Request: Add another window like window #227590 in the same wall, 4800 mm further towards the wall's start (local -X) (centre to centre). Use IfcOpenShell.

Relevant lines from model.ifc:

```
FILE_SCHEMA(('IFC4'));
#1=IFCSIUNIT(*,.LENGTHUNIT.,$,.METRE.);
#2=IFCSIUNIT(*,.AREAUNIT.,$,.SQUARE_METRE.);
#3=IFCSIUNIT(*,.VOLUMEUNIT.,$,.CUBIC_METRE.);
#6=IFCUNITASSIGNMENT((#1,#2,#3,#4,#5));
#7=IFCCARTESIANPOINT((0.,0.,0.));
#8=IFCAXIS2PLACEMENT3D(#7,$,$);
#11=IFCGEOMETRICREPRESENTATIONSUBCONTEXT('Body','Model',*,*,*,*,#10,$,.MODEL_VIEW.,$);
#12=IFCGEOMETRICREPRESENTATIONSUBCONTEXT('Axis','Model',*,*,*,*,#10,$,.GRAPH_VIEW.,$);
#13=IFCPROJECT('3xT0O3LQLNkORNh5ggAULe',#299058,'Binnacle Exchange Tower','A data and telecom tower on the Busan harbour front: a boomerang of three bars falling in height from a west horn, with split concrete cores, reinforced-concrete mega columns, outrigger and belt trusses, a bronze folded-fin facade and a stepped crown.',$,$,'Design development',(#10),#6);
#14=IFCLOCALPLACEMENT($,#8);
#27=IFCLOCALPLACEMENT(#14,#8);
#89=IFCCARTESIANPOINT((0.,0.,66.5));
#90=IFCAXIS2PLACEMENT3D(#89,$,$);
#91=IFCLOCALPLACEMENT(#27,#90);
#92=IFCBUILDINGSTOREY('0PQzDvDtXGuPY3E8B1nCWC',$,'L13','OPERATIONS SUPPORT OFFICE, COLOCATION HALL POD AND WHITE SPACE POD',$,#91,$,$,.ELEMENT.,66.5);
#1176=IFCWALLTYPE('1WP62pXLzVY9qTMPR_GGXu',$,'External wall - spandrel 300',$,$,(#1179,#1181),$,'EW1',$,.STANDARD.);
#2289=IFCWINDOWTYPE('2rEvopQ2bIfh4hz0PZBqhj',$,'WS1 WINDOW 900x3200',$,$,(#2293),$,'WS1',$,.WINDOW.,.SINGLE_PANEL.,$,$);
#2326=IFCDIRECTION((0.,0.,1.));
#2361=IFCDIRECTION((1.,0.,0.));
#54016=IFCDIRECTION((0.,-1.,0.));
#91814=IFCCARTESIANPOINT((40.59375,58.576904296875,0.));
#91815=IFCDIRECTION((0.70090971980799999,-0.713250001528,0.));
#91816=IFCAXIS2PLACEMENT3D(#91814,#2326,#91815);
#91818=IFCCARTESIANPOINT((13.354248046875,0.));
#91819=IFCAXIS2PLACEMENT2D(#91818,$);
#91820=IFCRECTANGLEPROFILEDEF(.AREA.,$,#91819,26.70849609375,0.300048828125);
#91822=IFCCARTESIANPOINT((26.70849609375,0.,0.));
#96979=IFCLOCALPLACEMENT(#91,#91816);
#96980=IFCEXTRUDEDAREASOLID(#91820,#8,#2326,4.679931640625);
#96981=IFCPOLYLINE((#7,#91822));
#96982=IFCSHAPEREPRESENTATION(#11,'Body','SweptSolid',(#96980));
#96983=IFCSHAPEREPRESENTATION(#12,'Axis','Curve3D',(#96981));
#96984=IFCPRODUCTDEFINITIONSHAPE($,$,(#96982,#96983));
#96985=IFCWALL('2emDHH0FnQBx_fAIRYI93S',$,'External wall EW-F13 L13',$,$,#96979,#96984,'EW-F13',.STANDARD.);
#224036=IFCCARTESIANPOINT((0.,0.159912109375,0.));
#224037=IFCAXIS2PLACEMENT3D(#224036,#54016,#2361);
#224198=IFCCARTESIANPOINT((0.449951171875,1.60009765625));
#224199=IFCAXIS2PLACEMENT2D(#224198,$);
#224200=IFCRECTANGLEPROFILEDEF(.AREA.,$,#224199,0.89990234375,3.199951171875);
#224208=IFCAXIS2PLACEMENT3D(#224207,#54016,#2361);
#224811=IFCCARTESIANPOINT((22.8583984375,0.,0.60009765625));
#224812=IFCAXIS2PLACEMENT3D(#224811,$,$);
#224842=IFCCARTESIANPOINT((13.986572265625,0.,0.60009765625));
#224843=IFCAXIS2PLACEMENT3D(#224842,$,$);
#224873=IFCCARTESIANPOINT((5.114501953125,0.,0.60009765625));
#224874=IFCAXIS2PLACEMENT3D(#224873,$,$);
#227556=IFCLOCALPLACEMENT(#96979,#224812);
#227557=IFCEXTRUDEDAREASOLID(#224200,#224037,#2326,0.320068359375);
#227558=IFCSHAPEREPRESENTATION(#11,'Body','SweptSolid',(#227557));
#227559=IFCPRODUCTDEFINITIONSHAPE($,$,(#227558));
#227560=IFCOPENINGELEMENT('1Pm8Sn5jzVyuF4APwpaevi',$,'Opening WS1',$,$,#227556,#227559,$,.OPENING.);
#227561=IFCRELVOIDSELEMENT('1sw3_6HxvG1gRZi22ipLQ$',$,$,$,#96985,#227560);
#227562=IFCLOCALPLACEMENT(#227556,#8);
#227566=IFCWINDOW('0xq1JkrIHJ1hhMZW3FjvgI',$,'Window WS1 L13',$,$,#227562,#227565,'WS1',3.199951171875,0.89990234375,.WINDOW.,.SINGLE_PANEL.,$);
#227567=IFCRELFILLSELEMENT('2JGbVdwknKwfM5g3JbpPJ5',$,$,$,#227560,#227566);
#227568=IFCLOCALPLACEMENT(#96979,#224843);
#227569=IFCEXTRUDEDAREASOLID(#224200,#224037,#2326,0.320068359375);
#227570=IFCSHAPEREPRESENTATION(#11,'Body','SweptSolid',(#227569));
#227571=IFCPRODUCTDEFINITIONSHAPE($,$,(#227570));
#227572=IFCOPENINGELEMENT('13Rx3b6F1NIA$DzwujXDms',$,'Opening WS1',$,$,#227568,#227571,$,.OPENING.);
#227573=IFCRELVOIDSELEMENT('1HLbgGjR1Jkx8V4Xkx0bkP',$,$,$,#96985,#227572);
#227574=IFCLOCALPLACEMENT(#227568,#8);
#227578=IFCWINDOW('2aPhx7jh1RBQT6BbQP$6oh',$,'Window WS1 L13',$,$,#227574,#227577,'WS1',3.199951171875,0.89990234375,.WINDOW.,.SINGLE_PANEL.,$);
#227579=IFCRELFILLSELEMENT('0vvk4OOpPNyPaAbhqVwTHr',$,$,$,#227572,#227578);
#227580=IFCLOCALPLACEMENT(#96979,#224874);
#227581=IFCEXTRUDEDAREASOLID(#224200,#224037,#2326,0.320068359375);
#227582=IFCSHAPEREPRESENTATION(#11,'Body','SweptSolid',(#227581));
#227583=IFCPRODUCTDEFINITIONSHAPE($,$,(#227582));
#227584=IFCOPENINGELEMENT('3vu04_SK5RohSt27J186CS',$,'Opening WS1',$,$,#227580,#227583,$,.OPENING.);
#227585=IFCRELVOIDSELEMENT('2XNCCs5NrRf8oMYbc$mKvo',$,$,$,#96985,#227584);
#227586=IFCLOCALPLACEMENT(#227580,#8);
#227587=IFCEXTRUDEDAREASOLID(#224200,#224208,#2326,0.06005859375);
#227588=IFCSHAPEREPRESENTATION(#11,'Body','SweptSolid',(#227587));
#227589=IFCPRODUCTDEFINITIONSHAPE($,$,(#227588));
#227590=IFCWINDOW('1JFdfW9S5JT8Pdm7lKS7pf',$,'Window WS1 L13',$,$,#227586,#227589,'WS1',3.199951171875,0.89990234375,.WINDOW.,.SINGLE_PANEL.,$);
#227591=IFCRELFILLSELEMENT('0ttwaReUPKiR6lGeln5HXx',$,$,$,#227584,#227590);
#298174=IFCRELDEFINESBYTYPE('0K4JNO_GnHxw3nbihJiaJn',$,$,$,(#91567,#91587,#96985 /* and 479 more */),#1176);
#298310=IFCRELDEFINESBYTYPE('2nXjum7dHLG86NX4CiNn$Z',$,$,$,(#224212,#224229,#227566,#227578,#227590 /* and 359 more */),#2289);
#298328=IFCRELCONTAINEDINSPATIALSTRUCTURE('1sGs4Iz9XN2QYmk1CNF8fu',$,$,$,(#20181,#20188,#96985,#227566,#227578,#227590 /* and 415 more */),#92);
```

```python
import ifcopenshell
import ifcopenshell.api.feature
import ifcopenshell.api.geometry
import ifcopenshell.api.root
import ifcopenshell.geom
import ifcopenshell.util.element
import ifcopenshell.util.placement
import ifcopenshell.util.shape
import ifcopenshell.util.unit

model = ifcopenshell.open("model.ifc")
unit_scale = ifcopenshell.util.unit.calculate_unit_scale(model)
settings = ifcopenshell.geom.settings()


def volume(element):
    """Net volume in cubic metres, openings subtracted."""
    shape = ifcopenshell.geom.create_shape(settings, element)
    return ifcopenshell.util.shape.get_volume(shape.geometry)


window = model.by_guid("1JFdfW9S5JT8Pdm7lKS7pf")
opening = window.FillsVoids[0].RelatingOpeningElement
wall = opening.VoidsElements[0].RelatingBuildingElement
before = volume(wall)
shift = ifcopenshell.util.placement.get_local_placement(wall.ObjectPlacement)[:3, 0] * -4.8 / unit_scale

# copy_class copies the void relationship, type, container and properties, but no geometry.
new_opening = ifcopenshell.api.root.copy_class(model, product=opening)
new_opening.Representation = ifcopenshell.util.element.copy_deep(
    model, opening.Representation, exclude=["IfcGeometricRepresentationContext", "IfcRepresentationMap"]
)
new_window = ifcopenshell.api.root.copy_class(model, product=window)
new_window.Representation = ifcopenshell.util.element.copy_deep(
    model, window.Representation, exclude=["IfcGeometricRepresentationContext", "IfcRepresentationMap"]
)
new_window.Tag = None
ifcopenshell.api.feature.add_filling(model, opening=new_opening, element=new_window)

for old, new in ((opening, new_opening), (window, new_window)):
    matrix = ifcopenshell.util.placement.get_local_placement(old.ObjectPlacement)
    matrix[:3, 3] += shift
    ifcopenshell.api.geometry.edit_object_placement(model, product=new, matrix=matrix, is_si=False)

after = volume(wall)

print(f"wall volume {before:.3f} -> {after:.3f} m3")

model.write("model_updated.ifc")
```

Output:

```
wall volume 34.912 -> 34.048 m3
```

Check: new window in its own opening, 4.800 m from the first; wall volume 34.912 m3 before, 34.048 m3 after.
